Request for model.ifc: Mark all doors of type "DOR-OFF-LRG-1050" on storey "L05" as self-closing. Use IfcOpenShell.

First a look at what the model holds.

```python
import ifcopenshell
import ifcopenshell.util.element

model = ifcopenshell.open("model.ifc")
print(model.schema)
storey = next(s for s in model.by_type("IfcBuildingStorey") if s.Name == "L05")
doors = [e for e in ifcopenshell.util.element.get_decomposition(storey) if e.is_a("IfcDoor")]
seen = {}
for e in doors:
    element_type = ifcopenshell.util.element.get_type(e)
    key = (element_type.Name if element_type != e and element_type else None, ifcopenshell.util.element.get_pset(e, "Pset_DoorCommon", "SelfClosing"))
    seen[key] = seen.get(key, 0) + 1
for (name, value), count in sorted(seen.items(), key=str):
    print(count, "x", name, "|", value)
```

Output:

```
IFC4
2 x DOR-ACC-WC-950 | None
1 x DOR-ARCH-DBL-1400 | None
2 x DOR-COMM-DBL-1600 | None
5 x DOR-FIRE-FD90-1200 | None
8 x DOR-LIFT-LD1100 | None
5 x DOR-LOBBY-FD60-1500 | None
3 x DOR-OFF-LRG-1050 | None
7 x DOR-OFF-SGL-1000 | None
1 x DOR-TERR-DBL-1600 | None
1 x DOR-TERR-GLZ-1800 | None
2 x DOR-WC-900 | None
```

```python
import ifcopenshell
import ifcopenshell.api.pset
import ifcopenshell.util.element

model = ifcopenshell.open("model.ifc")

storey = next(s for s in model.by_type("IfcBuildingStorey") if s.Name == "L05")
doors = [e for e in ifcopenshell.util.element.get_decomposition(storey) if e.is_a("IfcDoor")]

count = 0
for e in doors:
    element_type = ifcopenshell.util.element.get_type(e)
    if element_type in (None, e) or element_type.Name != "DOR-OFF-LRG-1050":
        continue
    # add_pset returns the element's existing set when there is one.
    pset = ifcopenshell.api.pset.add_pset(model, product=e, name="Pset_DoorCommon")
    ifcopenshell.api.pset.edit_pset(model, pset=pset, properties={"SelfClosing": True})
    count += 1

print(count, "doors updated")

model.write("model_edited.ifc")
```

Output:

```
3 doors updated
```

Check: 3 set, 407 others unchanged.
